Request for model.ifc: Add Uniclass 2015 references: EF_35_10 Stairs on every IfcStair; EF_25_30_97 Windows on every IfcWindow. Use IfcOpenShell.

First a look at what the model holds.

```python
import ifcopenshell

model = ifcopenshell.open("model.ifc")
print(model.schema)
print("classifications:", [c.Name for c in model.by_type("IfcClassification")])
for ifc_class in ("IfcDoor", "IfcRoof", "IfcStair", "IfcWall", "IfcWindow"):
    print(ifc_class, len(model.by_type(ifc_class)))
```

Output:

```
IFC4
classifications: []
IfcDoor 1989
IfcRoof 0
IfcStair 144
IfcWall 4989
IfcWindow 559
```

```python
import ifcopenshell
import ifcopenshell.api.classification

model = ifcopenshell.open("model.ifc")

system = ifcopenshell.api.classification.add_classification(model, classification="Uniclass 2015")

codes = {
    "IfcStair": ("EF_35_10", "Stairs"),
    "IfcWindow": ("EF_25_30_97", "Windows"),
}
for ifc_class, (code, name) in codes.items():
    products = model.by_type(ifc_class)
    ifcopenshell.api.classification.add_reference(
        model, products=products, classification=system, identification=code, name=name
    )
    print(code, len(products))

model.write("model_edited.ifc")
```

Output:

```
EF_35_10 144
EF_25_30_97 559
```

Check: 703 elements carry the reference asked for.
